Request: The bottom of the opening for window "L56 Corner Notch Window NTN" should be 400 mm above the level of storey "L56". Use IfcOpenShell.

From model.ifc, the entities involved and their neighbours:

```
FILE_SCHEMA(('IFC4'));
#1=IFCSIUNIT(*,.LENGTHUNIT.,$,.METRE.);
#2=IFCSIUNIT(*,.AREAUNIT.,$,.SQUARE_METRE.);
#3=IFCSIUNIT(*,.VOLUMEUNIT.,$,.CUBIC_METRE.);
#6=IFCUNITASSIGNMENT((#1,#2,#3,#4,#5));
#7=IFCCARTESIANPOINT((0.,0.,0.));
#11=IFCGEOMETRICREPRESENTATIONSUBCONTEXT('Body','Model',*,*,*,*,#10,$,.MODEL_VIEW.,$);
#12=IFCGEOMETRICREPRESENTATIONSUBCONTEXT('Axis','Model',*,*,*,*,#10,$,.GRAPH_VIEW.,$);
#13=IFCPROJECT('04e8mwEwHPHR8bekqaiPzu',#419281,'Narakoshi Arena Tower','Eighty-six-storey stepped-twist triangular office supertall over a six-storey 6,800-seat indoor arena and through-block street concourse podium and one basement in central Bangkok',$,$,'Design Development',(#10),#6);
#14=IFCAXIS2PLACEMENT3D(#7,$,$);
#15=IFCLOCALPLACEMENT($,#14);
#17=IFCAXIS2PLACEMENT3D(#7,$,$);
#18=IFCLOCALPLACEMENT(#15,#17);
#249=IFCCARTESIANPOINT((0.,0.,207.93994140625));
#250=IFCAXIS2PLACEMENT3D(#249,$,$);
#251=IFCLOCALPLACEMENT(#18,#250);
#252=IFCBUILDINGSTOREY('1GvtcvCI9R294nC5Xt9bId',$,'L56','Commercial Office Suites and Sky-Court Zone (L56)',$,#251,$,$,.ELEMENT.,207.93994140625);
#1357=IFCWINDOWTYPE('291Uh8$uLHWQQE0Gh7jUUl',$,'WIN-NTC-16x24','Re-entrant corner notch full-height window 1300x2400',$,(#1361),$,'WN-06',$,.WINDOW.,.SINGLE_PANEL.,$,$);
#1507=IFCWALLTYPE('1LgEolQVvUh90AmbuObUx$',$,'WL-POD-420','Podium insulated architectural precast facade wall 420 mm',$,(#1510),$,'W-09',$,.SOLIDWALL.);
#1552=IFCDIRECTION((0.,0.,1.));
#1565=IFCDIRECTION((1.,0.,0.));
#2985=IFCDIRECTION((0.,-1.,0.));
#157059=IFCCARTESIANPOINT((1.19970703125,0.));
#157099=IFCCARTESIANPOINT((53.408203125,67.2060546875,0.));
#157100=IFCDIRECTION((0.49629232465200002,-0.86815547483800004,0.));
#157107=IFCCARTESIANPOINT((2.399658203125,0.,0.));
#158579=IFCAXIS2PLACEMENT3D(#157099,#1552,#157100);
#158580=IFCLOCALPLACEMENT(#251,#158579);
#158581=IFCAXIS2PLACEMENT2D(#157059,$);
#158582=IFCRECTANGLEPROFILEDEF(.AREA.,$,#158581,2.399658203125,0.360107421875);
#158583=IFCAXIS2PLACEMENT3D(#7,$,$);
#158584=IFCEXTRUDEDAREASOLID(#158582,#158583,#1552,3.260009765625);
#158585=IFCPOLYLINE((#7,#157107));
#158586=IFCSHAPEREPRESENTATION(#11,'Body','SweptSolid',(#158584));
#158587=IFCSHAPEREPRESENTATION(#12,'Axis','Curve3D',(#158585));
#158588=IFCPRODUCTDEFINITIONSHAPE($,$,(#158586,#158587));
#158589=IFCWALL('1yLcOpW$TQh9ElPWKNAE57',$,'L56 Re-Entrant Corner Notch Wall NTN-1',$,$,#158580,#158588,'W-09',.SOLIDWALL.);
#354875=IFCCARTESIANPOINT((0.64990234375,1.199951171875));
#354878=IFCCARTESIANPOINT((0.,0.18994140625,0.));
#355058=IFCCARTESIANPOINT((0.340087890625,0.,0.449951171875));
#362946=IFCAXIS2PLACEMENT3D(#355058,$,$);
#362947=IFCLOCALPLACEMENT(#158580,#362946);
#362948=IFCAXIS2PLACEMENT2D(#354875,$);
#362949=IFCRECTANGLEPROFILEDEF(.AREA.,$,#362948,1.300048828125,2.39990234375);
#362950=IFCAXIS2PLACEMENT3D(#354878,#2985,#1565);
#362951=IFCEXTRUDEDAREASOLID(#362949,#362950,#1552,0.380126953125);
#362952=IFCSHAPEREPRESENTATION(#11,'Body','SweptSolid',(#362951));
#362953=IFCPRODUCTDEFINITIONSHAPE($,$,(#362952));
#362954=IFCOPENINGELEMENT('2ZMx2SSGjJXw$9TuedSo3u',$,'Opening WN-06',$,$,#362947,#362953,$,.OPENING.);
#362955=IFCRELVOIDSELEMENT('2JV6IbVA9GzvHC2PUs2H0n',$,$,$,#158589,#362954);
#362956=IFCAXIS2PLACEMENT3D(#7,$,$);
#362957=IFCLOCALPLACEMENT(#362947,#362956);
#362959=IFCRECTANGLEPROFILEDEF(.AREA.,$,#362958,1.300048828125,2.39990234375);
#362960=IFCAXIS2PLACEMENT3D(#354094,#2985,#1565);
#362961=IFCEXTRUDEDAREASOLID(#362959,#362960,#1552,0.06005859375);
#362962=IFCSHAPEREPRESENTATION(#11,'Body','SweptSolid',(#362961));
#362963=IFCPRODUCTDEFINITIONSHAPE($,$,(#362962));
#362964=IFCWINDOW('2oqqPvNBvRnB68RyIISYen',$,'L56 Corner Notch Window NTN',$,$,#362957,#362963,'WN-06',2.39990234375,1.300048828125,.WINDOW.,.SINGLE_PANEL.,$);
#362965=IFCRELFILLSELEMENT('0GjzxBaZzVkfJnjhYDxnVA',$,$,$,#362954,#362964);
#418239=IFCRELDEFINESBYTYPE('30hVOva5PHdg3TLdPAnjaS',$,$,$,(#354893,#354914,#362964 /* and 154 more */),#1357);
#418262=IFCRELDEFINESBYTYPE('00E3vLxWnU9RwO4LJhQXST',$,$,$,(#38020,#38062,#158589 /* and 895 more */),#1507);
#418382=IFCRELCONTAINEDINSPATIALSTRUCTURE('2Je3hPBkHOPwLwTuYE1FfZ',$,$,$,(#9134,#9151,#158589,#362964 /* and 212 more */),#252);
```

```python
import numpy as np
import ifcopenshell
import ifcopenshell.api.geometry
import ifcopenshell.geom
import ifcopenshell.util.element
import ifcopenshell.util.placement
import ifcopenshell.util.shape
import ifcopenshell.util.unit

model = ifcopenshell.open("model.ifc")
unit_scale = ifcopenshell.util.unit.calculate_unit_scale(model)

window = model.by_id(362964)
opening = window.FillsVoids[0].RelatingOpeningElement
storey = ifcopenshell.util.element.get_container(window, ifc_class="IfcBuildingStorey")
level = ifcopenshell.util.placement.get_local_placement(storey.ObjectPlacement)[2, 3]

# The opening's origin need not be at the sill, so measure its lowest point.
shape = ifcopenshell.geom.create_shape(ifcopenshell.geom.settings(), opening)
bottom = ifcopenshell.util.shape.get_shape_bottom_elevation(shape, shape.geometry) / unit_scale
dz = level + 0.4 / unit_scale - bottom

shift = np.array([0.0, 0.0, dz])
# The window is placed relative to its opening, so it follows when the opening moves.
matrix = ifcopenshell.util.placement.get_local_placement(opening.ObjectPlacement)
matrix[:3, 3] += shift
ifcopenshell.api.geometry.edit_object_placement(
    model, product=opening, matrix=matrix, is_si=False, should_transform_children=True
)

print(f"moved by {dz * unit_scale:+.3f} m")

model.write("model_edited.ifc")
```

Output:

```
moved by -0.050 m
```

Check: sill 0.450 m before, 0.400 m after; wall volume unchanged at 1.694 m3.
